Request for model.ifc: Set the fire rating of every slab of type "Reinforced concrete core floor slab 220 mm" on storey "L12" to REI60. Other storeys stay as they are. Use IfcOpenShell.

First a look at what the model holds.

```python
import ifcopenshell
import ifcopenshell.util.element

model = ifcopenshell.open("model.ifc")
print(model.schema)
storey = next(s for s in model.by_type("IfcBuildingStorey") if s.Name == "L12")
slabs = [e for e in ifcopenshell.util.element.get_decomposition(storey) if e.is_a("IfcSlab")]
seen = {}
for e in slabs:
    element_type = ifcopenshell.util.element.get_type(e)
    key = (element_type.Name if element_type != e and element_type else None, ifcopenshell.util.element.get_pset(e, "Pset_SlabCommon", "FireRating"))
    seen[key] = seen.get(key, 0) + 1
for (name, value), count in sorted(seen.items(), key=str):
    print(count, "x", name, "|", value)
```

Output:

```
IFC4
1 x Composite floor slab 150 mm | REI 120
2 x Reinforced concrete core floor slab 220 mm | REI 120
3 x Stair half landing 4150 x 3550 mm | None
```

```python
import ifcopenshell
import ifcopenshell.api.pset
import ifcopenshell.util.element

model = ifcopenshell.open("model.ifc")

storey = next(s for s in model.by_type("IfcBuildingStorey") if s.Name == "L12")
slabs = [e for e in ifcopenshell.util.element.get_decomposition(storey) if e.is_a("IfcSlab")]

count = 0
for e in slabs:
    element_type = ifcopenshell.util.element.get_type(e)
    if element_type in (None, e) or element_type.Name != "Reinforced concrete core floor slab 220 mm":
        continue
    # add_pset returns the element's existing set when there is one.
    pset = ifcopenshell.api.pset.add_pset(model, product=e, name="Pset_SlabCommon")
    ifcopenshell.api.pset.edit_pset(model, pset=pset, properties={"FireRating": "REI60"})
    count += 1

print(count, "slabs updated")

model.write("model_v2.ifc")
```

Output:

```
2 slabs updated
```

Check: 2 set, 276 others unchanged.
